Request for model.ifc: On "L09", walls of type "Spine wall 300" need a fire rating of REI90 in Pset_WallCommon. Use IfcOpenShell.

First a look at what the model holds.

```python
import ifcopenshell
import ifcopenshell.util.element

model = ifcopenshell.open("model.ifc")
print(model.schema)
storey = next(s for s in model.by_type("IfcBuildingStorey") if s.Name == "L09")
walls = [e for e in ifcopenshell.util.element.get_decomposition(storey) if e.is_a("IfcWall")]
seen = {}
for e in walls:
    element_type = ifcopenshell.util.element.get_type(e)
    key = (element_type.Name if element_type != e and element_type else None, ifcopenshell.util.element.get_pset(e, "Pset_WallCommon", "FireRating"))
    seen[key] = seen.get(key, 0) + 1
for (name, value), count in sorted(seen.items(), key=str):
    print(count, "x", name, "|", value)
```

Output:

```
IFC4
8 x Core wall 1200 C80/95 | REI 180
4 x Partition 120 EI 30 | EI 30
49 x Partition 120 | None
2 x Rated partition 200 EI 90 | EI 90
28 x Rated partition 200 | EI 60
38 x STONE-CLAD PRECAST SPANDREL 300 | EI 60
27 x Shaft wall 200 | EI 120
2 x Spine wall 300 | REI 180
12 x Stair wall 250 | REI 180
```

```python
import ifcopenshell
import ifcopenshell.api.pset
import ifcopenshell.util.element

model = ifcopenshell.open("model.ifc")

storey = next(s for s in model.by_type("IfcBuildingStorey") if s.Name == "L09")
walls = [e for e in ifcopenshell.util.element.get_decomposition(storey) if e.is_a("IfcWall")]

count = 0
for e in walls:
    element_type = ifcopenshell.util.element.get_type(e)
    if element_type in (None, e) or element_type.Name != "Spine wall 300":
        continue
    found = ifcopenshell.util.element.get_pset(e, "Pset_WallCommon", should_inherit=False)
    if found:
        pset = model.by_id(found["id"])
        if len(ifcopenshell.util.element.get_elements_by_pset(pset)) > 1:
            pset = ifcopenshell.api.pset.unshare_pset(model, products=[e], pset=pset)[0]
    else:
        pset = ifcopenshell.api.pset.add_pset(model, product=e, name="Pset_WallCommon")
    ifcopenshell.api.pset.edit_pset(model, pset=pset, properties={"FireRating": "REI90"})
    count += 1

print(count, "walls updated")

model.write("model_updated.ifc")
```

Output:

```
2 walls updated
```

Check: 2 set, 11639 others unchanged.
